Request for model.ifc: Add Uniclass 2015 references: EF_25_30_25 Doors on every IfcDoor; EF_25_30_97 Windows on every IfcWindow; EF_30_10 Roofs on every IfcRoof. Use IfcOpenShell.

First a look at what the model holds.

```python
import ifcopenshell

model = ifcopenshell.open("model.ifc")
print(model.schema)
print("classifications:", [c.Name for c in model.by_type("IfcClassification")])
for ifc_class in ("IfcDoor", "IfcRoof", "IfcStair", "IfcWall", "IfcWindow"):
    print(ifc_class, len(model.by_type(ifc_class)))
```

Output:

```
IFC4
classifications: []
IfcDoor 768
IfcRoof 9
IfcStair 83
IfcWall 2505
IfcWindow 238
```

```python
import ifcopenshell
import ifcopenshell.api.classification

model = ifcopenshell.open("model.ifc")

system = ifcopenshell.api.classification.add_classification(model, classification="Uniclass 2015")

codes = {
    "IfcDoor": ("EF_25_30_25", "Doors"),
    "IfcWindow": ("EF_25_30_97", "Windows"),
    "IfcRoof": ("EF_30_10", "Roofs"),
}
for ifc_class, (code, name) in codes.items():
    products = model.by_type(ifc_class)
    ifcopenshell.api.classification.add_reference(
        model, products=products, classification=system, identification=code, name=name
    )
    print(code, len(products))

model.write("model_rev.ifc")
```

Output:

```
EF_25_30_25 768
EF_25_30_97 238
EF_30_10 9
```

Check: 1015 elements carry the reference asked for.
